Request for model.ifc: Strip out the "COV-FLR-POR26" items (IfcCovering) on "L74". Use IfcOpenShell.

First a look at what the model holds.

```python
import ifcopenshell
import ifcopenshell.util.element

model = ifcopenshell.open("model.ifc")
print(model.schema)
storey = next(s for s in model.by_type("IfcBuildingStorey") if s.Name == "L74")
coverings = [e for e in ifcopenshell.util.element.get_decomposition(storey) if e.is_a("IfcCovering")]
seen = {}
for e in coverings:
    element_type = ifcopenshell.util.element.get_type(e)
    name = element_type.Name if element_type not in (None, e) else None
    seen[name] = seen.get(name, 0) + 1
for name, count in sorted(seen.items(), key=str):
    print(count, "x", name)
```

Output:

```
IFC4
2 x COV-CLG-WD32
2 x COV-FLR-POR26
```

```python
import ifcopenshell
import ifcopenshell.api.root
import ifcopenshell.util.element

model = ifcopenshell.open("model.ifc")

storey = next(s for s in model.by_type("IfcBuildingStorey") if s.Name == "L74")
coverings = [e for e in ifcopenshell.util.element.get_decomposition(storey) if e.is_a("IfcCovering")]
targets = [e for e in coverings if (t := ifcopenshell.util.element.get_type(e)) not in (None, e) and t.Name == "COV-FLR-POR26"]

for e in targets:
    ifcopenshell.api.root.remove_product(model, product=e)
print(len(targets), "removed")

model.write("model_v2.ifc")
```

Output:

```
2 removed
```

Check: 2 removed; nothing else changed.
